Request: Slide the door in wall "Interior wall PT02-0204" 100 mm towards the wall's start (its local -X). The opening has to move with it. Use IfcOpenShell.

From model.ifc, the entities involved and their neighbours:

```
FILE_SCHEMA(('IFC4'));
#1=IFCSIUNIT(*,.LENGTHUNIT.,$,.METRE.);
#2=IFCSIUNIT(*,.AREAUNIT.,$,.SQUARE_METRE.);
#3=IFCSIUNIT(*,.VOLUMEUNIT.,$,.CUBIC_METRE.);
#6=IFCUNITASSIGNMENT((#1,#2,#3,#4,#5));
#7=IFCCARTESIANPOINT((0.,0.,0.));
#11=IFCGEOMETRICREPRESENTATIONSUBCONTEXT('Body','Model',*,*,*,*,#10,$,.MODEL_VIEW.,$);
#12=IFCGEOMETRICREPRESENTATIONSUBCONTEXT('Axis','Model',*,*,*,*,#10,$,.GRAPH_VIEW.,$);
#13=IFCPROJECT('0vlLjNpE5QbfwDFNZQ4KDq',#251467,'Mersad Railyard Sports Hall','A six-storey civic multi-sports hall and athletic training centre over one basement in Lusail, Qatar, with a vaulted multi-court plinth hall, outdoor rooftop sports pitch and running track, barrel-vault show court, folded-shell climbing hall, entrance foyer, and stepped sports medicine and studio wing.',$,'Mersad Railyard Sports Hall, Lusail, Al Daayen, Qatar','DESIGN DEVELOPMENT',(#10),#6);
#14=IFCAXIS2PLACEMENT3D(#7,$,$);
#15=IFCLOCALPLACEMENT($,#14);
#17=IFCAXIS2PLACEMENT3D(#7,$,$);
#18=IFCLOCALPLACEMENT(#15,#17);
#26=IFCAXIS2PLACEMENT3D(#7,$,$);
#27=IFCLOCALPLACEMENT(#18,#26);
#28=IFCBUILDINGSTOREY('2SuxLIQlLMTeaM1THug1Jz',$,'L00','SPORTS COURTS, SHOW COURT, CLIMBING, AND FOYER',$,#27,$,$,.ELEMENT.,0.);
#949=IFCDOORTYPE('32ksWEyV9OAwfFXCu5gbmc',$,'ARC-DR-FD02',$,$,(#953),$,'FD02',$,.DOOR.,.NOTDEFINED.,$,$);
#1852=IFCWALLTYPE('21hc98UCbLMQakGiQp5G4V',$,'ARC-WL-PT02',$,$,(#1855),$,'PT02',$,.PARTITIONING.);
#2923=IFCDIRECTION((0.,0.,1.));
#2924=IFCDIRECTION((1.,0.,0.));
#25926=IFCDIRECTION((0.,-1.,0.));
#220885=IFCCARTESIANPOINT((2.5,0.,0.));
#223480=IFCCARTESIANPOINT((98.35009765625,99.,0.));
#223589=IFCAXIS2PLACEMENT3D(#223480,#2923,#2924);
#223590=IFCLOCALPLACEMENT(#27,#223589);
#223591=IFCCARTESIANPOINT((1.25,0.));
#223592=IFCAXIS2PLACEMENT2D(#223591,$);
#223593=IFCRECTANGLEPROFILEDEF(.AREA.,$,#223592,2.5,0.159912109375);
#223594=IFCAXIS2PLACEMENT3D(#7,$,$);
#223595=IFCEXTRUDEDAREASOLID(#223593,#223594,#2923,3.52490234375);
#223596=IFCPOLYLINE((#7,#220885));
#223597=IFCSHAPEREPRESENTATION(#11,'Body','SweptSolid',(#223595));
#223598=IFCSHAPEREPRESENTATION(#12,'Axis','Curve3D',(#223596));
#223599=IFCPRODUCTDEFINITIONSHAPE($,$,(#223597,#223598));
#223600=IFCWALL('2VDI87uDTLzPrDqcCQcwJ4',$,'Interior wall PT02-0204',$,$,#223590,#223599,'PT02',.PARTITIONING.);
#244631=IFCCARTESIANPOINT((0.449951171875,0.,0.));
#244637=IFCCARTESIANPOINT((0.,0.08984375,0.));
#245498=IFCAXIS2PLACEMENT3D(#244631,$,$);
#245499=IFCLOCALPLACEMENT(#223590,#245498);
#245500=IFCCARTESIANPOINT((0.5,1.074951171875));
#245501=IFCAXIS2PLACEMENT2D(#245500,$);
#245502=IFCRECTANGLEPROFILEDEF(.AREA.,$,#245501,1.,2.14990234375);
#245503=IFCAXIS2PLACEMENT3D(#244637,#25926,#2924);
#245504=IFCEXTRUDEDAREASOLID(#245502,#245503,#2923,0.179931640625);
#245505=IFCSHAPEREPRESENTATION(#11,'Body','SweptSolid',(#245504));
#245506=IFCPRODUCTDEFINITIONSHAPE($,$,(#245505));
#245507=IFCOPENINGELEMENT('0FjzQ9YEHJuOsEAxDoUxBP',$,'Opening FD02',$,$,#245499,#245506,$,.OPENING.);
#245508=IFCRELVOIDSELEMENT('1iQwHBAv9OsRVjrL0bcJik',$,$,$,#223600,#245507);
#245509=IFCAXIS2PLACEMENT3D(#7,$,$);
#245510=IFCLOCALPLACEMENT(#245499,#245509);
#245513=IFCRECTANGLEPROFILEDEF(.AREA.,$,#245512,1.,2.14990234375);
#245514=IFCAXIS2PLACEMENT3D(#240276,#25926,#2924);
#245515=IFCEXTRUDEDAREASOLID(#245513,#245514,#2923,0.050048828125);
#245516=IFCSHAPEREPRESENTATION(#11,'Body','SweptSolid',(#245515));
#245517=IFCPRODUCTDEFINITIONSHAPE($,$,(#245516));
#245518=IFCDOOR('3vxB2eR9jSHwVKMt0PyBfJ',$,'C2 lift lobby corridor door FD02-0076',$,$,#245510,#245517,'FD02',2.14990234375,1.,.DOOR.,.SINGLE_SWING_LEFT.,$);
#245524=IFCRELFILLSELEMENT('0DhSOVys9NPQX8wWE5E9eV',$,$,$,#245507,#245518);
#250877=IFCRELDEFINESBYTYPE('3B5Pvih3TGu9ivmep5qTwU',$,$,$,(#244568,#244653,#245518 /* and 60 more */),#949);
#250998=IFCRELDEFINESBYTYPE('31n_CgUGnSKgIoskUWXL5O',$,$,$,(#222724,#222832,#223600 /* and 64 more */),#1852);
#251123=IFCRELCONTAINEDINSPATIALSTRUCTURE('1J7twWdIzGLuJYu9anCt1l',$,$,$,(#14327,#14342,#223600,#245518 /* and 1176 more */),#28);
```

```python
import ifcopenshell
import ifcopenshell.api.geometry
import ifcopenshell.util.placement
import ifcopenshell.util.unit

model = ifcopenshell.open("model.ifc")
unit_scale = ifcopenshell.util.unit.calculate_unit_scale(model)

door = model.by_guid("3vxB2eR9jSHwVKMt0PyBfJ")
opening = door.FillsVoids[0].RelatingOpeningElement
wall = opening.VoidsElements[0].RelatingBuildingElement

wall_matrix = ifcopenshell.util.placement.get_local_placement(wall.ObjectPlacement)
shift = wall_matrix[:3, 0] * -0.1 / unit_scale
before = ifcopenshell.util.placement.get_local_placement(door.ObjectPlacement)[:3, 3].copy()

# The door is placed relative to its opening, so it follows when the opening moves.
matrix = ifcopenshell.util.placement.get_local_placement(opening.ObjectPlacement)
matrix[:3, 3] += shift
ifcopenshell.api.geometry.edit_object_placement(
    model, product=opening, matrix=matrix, is_si=False, should_transform_children=True
)

after = ifcopenshell.util.placement.get_local_placement(door.ObjectPlacement)[:3, 3]
print("door moved by", (after - before).round(3) + 0.0)

model.write("model-out.ifc")
```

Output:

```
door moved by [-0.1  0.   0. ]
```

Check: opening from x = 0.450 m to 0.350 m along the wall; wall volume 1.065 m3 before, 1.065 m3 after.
